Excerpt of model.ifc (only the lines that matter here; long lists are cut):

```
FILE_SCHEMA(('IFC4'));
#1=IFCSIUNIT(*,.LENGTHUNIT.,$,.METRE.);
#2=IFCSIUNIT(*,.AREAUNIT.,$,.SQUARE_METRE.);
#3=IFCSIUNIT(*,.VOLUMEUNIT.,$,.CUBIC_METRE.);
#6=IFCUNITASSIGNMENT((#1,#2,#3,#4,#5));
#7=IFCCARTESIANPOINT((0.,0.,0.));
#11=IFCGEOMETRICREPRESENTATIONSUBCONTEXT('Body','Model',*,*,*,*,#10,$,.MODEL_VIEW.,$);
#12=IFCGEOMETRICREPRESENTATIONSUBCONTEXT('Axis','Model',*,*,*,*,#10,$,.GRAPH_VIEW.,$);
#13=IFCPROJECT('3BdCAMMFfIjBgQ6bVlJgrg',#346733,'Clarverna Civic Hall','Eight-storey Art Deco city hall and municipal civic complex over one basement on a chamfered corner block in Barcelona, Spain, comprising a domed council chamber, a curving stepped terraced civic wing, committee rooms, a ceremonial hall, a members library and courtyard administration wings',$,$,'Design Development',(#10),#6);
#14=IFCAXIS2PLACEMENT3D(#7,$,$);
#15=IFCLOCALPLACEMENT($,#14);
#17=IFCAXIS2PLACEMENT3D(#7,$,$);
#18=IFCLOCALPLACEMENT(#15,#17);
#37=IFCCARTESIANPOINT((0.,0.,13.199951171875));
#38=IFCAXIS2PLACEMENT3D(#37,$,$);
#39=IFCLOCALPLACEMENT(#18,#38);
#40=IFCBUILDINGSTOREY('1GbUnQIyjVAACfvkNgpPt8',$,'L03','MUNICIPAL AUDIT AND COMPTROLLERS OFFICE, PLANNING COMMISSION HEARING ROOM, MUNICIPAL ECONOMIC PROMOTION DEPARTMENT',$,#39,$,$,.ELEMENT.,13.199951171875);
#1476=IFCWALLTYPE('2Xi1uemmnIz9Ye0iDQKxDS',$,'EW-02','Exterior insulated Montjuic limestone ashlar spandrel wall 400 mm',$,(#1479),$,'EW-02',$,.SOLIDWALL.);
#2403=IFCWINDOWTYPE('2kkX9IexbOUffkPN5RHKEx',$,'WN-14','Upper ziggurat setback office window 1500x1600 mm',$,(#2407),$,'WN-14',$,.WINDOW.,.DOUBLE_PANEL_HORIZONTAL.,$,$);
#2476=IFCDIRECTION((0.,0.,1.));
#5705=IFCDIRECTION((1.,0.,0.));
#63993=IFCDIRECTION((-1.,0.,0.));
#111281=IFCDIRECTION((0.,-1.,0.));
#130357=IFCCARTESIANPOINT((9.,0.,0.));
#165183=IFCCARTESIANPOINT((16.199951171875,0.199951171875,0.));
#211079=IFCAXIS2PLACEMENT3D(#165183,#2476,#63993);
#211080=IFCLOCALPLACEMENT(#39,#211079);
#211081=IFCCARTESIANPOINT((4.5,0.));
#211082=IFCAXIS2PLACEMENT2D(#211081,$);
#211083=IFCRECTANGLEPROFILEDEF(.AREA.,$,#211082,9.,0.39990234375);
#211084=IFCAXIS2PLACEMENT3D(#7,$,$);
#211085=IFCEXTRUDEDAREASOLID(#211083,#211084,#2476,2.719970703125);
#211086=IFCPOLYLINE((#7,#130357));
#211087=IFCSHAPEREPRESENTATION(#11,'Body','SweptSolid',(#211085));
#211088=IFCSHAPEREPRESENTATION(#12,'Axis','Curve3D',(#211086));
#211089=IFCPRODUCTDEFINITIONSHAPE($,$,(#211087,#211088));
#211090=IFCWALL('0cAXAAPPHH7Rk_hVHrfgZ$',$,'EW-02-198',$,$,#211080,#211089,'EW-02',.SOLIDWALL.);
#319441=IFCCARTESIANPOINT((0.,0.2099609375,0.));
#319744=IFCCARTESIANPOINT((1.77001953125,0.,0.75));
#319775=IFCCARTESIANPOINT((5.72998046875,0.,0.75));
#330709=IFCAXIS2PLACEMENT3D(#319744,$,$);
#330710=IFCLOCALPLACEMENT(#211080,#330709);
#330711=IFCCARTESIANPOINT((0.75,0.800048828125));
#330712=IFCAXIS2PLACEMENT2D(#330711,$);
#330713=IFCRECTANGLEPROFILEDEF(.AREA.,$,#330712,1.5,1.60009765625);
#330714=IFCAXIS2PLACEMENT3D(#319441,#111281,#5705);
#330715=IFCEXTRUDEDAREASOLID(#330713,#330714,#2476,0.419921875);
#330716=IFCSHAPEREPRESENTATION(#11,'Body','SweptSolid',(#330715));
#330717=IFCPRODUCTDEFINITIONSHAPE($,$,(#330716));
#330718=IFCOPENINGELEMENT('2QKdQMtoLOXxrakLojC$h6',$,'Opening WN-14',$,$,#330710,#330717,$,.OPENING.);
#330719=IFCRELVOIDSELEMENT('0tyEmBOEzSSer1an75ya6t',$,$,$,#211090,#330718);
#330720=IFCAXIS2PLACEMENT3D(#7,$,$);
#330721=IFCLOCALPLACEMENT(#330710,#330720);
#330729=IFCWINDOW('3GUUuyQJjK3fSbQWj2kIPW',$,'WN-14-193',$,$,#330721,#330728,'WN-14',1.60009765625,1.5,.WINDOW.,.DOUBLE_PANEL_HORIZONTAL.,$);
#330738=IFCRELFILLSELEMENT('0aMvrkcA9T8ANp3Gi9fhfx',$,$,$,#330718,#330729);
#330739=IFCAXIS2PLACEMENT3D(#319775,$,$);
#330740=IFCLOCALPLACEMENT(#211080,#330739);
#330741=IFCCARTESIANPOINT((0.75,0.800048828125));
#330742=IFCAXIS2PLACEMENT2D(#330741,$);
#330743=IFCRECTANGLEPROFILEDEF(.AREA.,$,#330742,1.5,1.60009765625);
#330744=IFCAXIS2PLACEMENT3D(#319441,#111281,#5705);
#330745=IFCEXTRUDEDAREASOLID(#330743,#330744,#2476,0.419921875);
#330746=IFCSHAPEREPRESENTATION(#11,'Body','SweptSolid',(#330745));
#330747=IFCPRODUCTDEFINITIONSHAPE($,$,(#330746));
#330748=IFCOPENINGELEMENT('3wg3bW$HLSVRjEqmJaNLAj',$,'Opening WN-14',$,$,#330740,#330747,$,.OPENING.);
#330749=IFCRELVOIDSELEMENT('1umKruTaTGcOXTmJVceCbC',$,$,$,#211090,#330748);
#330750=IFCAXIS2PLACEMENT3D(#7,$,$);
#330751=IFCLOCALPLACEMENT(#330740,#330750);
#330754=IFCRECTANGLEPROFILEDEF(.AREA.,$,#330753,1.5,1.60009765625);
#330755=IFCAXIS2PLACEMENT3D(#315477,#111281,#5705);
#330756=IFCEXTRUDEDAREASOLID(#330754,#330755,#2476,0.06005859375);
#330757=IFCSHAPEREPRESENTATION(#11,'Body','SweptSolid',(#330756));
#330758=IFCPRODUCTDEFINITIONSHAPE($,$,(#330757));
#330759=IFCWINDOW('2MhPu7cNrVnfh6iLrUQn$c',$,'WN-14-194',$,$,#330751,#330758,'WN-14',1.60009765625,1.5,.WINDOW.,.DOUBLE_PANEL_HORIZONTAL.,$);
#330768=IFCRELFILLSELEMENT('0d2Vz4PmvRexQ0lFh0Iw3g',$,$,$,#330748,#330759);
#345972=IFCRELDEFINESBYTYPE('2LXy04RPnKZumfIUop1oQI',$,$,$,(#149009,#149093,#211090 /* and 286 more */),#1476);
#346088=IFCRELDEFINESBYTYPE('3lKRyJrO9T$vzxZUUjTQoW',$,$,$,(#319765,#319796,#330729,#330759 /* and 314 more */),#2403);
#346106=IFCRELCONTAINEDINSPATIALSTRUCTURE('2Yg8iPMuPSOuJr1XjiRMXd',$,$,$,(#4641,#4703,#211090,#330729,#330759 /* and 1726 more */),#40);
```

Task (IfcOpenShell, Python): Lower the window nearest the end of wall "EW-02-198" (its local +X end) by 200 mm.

```python
import numpy as np
import ifcopenshell
import ifcopenshell.api.geometry
import ifcopenshell.util.placement
import ifcopenshell.util.unit

model = ifcopenshell.open("model.ifc")
unit_scale = ifcopenshell.util.unit.calculate_unit_scale(model)

window = model.by_guid("2MhPu7cNrVnfh6iLrUQn$c")
opening = window.FillsVoids[0].RelatingOpeningElement
dz = -0.2 / unit_scale

shift = np.array([0.0, 0.0, dz])
# The window is placed relative to its opening, so it follows when the opening moves.
matrix = ifcopenshell.util.placement.get_local_placement(opening.ObjectPlacement)
matrix[:3, 3] += shift
ifcopenshell.api.geometry.edit_object_placement(
    model, product=opening, matrix=matrix, is_si=False, should_transform_children=True
)

print(f"moved by {dz * unit_scale:+.3f} m")

model.write("model_v2.ifc")
```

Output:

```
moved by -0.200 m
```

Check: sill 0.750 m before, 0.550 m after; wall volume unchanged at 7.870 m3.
